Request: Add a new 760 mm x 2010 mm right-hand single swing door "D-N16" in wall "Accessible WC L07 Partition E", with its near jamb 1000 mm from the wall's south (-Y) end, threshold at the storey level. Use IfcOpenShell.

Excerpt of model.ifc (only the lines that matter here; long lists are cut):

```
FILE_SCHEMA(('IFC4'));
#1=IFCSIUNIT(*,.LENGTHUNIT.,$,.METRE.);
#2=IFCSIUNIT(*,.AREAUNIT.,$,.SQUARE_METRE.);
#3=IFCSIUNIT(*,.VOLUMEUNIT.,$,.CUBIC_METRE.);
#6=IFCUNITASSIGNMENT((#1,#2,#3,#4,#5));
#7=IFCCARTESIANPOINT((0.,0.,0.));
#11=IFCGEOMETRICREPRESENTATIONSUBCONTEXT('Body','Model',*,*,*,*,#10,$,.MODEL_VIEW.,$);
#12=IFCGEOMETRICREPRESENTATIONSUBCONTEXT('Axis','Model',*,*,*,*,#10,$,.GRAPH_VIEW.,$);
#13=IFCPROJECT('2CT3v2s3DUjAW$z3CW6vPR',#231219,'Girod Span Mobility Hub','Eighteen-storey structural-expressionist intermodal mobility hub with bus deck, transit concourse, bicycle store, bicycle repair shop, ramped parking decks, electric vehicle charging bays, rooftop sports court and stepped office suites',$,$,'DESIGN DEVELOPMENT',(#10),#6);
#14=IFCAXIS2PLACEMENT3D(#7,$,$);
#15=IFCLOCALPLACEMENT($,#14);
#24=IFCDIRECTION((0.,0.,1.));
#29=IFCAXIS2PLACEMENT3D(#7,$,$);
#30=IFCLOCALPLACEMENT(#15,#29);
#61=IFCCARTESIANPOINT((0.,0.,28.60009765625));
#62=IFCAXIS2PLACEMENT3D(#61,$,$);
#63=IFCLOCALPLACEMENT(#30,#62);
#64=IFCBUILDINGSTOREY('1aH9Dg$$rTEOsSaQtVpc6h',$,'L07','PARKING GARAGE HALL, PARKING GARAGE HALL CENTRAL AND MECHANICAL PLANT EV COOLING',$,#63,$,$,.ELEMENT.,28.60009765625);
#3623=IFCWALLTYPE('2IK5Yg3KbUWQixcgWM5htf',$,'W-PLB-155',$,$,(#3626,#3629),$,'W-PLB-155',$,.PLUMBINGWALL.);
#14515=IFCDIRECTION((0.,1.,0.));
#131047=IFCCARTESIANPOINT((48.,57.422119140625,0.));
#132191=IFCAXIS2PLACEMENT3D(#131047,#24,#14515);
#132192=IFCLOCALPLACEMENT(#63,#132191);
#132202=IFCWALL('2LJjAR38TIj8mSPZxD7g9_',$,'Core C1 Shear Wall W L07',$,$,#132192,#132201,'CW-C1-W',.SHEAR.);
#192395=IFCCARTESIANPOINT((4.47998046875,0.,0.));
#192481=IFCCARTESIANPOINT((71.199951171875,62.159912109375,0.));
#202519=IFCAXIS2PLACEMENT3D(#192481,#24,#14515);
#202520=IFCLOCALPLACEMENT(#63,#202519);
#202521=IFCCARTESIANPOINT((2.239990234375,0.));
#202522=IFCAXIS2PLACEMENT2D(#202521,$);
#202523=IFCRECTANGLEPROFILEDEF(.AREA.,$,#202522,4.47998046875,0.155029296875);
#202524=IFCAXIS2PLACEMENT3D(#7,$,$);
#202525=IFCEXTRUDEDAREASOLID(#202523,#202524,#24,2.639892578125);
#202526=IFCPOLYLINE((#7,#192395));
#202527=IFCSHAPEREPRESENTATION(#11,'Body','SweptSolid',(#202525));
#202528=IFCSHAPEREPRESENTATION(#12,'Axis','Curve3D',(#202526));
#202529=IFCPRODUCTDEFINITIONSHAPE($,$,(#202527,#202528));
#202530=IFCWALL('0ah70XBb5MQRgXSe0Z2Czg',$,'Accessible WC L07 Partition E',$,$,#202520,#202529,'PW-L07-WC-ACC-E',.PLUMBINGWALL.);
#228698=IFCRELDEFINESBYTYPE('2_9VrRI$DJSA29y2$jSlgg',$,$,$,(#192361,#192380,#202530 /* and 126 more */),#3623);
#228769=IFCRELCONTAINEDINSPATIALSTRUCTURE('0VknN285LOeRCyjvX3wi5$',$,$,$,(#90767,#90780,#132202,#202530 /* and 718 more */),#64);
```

```python
import numpy as np
import ifcopenshell
import ifcopenshell.api.feature
import ifcopenshell.api.geometry
import ifcopenshell.api.root
import ifcopenshell.api.spatial
import ifcopenshell.geom
import ifcopenshell.util.element
import ifcopenshell.util.placement
import ifcopenshell.util.representation
import ifcopenshell.util.shape
import ifcopenshell.util.unit

model = ifcopenshell.open("model.ifc")
unit_scale = ifcopenshell.util.unit.calculate_unit_scale(model)
settings = ifcopenshell.geom.settings()


def volume(element):
    """Net volume in cubic metres, openings subtracted."""
    shape = ifcopenshell.geom.create_shape(settings, element)
    return ifcopenshell.util.shape.get_volume(shape.geometry)


wall = model.by_id(202530)
storey = ifcopenshell.util.element.get_container(wall, ifc_class="IfcBuildingStorey")
context = ifcopenshell.util.representation.get_context(model, "Model", "Body", "MODEL_VIEW")
before = volume(wall)

width, height, from_end, sill = 0.76, 2.01, 1, 0.0  # metres

# The wall runs along its own X axis, and the end named is its -X end.
wall_shape = ifcopenshell.geom.create_shape(settings, wall)
x, y, z = ifcopenshell.util.shape.get_vertices(wall_shape.geometry).T
start = x.min() + from_end
face, thickness = float(y.min()), float(y.max() - y.min())
wall_matrix = ifcopenshell.util.placement.get_local_placement(wall.ObjectPlacement)
level = ifcopenshell.util.placement.get_local_placement(storey.ObjectPlacement)[2, 3]


def in_wall(x, y):
    """Placement at x, y metres in the wall's axes, at sill height."""
    matrix = wall_matrix.copy()
    matrix[:, 3] = wall_matrix @ np.array([x / unit_scale, y / unit_scale, 0.0, 1.0])
    matrix[2, 3] = level + sill / unit_scale
    return matrix


# Opening: a box that overshoots both wall faces by 50 mm.
opening = ifcopenshell.api.root.create_entity(model, ifc_class="IfcOpeningElement", predefined_type="OPENING")
box = ifcopenshell.api.geometry.add_wall_representation(
    model, context=context, length=width, height=height, thickness=thickness + 0.1
)
ifcopenshell.api.geometry.assign_representation(model, product=opening, representation=box)
ifcopenshell.api.geometry.edit_object_placement(model, product=opening, matrix=in_wall(start, face - 0.05), is_si=False)
ifcopenshell.api.feature.add_feature(model, feature=opening, element=wall)

door = ifcopenshell.api.root.create_entity(model, ifc_class="IfcDoor", name="D-N16", predefined_type="DOOR")
door.OverallWidth, door.OverallHeight = width / unit_scale, height / unit_scale
door.OperationType = "SINGLE_SWING_RIGHT"
body = ifcopenshell.api.geometry.add_door_representation(
    model,
    context=context,
    overall_width=door.OverallWidth,
    overall_height=door.OverallHeight,
    operation_type="SINGLE_SWING_RIGHT",
    lining_properties={"LiningDepth": thickness / unit_scale, "ThresholdDepth": thickness / unit_scale},
)
ifcopenshell.api.geometry.assign_representation(model, product=door, representation=body)
ifcopenshell.api.spatial.assign_container(model, products=[door], relating_structure=storey)
ifcopenshell.api.feature.add_filling(model, opening=opening, element=door)

# The lining spans the wall, so the door starts at the wall face.
ifcopenshell.api.geometry.edit_object_placement(model, product=door, matrix=in_wall(start, face), is_si=False)

after = volume(wall)

print(f"wall volume {before:.3f} -> {after:.3f} m3")

model.write("model_rev.ifc")
```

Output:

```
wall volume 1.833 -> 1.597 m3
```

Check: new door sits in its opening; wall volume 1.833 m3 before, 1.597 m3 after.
